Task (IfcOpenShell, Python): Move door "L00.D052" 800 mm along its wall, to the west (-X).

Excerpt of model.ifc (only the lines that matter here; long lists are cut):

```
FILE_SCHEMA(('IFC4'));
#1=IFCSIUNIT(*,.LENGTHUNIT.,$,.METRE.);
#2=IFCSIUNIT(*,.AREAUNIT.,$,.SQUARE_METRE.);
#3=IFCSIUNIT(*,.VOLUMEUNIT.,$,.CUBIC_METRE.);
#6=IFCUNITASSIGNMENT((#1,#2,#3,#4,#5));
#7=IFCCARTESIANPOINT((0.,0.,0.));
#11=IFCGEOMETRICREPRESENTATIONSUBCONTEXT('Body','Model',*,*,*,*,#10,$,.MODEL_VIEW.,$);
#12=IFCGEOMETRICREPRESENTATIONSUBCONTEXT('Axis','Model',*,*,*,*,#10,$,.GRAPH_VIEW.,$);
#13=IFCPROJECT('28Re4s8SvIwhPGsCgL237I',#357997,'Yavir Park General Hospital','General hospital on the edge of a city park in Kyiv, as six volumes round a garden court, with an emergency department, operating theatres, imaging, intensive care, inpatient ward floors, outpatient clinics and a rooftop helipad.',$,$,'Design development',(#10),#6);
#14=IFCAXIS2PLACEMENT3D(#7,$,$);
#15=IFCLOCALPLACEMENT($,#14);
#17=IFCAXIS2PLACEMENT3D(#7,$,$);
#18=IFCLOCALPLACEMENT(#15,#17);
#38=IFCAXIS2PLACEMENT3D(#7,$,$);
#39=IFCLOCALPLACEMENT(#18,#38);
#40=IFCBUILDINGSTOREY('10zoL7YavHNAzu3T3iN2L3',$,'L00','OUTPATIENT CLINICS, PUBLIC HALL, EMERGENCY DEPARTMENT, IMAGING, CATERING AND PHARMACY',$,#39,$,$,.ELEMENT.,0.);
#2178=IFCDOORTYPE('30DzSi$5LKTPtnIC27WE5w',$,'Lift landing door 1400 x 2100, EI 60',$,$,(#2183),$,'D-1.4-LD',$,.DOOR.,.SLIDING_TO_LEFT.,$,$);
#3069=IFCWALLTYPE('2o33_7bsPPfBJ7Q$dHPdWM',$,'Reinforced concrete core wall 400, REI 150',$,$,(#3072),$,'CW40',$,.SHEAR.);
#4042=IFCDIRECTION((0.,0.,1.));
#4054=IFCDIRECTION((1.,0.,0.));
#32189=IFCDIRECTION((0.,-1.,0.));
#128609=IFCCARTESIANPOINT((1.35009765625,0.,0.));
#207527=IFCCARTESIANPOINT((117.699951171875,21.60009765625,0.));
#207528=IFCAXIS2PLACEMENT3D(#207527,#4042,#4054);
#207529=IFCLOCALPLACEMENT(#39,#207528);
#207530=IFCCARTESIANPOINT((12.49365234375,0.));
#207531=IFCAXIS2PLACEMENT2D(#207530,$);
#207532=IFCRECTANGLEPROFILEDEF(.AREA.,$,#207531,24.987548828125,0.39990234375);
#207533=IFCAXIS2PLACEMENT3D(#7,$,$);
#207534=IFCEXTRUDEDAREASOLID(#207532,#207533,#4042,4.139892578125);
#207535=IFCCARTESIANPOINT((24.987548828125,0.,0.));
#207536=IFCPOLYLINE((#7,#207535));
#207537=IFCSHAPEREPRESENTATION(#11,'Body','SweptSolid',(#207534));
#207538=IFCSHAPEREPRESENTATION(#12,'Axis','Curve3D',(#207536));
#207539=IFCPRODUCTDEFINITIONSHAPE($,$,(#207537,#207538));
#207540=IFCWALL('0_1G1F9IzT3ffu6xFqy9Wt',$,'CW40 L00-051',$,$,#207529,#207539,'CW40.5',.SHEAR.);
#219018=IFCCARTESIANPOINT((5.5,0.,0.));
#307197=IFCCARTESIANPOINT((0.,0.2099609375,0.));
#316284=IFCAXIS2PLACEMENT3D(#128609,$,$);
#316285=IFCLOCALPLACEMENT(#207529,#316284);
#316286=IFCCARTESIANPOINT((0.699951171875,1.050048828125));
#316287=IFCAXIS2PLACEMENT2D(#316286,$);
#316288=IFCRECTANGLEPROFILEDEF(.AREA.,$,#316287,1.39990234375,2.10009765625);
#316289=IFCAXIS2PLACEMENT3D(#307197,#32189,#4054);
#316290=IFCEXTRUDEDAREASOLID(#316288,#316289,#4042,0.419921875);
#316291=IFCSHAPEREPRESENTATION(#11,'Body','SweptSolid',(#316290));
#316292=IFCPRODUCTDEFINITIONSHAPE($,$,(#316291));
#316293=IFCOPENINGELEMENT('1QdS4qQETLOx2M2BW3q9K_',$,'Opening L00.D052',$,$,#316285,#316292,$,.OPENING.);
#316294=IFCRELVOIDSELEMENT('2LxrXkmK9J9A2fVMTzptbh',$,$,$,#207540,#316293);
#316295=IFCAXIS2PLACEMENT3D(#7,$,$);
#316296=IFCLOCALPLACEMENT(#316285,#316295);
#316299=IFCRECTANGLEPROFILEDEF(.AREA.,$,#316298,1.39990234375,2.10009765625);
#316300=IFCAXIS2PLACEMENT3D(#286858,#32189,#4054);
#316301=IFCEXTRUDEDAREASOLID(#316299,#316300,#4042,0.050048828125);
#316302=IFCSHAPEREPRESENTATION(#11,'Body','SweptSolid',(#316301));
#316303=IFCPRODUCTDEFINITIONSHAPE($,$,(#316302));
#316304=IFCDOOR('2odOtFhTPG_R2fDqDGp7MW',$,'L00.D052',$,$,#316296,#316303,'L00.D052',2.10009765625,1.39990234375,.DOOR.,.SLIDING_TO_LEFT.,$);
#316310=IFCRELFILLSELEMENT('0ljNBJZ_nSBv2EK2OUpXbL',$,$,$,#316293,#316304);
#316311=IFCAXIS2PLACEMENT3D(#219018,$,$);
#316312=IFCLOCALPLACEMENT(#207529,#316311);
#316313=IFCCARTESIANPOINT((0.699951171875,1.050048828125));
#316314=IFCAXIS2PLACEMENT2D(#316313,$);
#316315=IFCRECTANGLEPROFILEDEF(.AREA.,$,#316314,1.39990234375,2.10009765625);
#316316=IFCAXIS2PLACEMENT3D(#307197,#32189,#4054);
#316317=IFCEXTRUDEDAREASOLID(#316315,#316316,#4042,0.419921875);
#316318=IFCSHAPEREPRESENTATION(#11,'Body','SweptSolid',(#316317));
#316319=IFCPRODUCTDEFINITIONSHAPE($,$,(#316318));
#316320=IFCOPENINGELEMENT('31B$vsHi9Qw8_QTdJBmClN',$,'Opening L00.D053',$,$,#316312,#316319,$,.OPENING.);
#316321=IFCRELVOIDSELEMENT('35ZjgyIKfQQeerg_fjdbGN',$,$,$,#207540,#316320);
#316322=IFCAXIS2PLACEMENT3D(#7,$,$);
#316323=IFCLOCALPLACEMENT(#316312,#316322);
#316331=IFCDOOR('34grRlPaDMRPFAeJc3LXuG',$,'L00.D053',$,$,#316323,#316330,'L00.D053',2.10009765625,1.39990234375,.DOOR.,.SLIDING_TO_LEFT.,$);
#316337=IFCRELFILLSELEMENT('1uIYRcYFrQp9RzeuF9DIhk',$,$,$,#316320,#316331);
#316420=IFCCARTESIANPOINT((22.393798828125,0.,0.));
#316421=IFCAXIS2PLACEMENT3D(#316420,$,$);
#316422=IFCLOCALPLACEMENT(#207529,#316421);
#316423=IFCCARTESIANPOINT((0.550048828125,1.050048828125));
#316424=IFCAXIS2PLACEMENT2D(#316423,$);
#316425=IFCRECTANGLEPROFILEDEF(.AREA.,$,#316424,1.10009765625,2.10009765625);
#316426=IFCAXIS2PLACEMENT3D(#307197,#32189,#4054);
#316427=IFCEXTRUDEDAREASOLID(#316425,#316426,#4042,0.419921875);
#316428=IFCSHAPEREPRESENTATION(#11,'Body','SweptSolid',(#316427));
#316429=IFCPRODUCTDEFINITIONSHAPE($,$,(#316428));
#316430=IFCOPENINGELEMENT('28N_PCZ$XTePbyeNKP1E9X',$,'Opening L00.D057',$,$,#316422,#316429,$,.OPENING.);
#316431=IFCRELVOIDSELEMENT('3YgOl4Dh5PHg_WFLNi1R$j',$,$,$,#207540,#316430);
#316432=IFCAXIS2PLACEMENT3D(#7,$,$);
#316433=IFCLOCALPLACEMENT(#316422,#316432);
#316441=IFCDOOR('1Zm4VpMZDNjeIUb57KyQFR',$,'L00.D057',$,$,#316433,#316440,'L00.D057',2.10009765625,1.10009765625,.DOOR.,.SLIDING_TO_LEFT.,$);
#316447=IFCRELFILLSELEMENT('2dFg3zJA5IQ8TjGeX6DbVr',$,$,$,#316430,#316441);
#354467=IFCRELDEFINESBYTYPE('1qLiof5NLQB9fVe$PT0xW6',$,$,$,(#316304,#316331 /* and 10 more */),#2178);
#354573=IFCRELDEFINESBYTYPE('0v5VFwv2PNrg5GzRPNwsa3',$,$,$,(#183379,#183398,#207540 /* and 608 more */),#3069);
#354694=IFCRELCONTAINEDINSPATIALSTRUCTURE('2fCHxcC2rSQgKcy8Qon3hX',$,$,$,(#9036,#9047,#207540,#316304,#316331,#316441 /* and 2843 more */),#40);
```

```python
import ifcopenshell
import ifcopenshell.api.geometry
import ifcopenshell.util.placement
import ifcopenshell.util.unit

model = ifcopenshell.open("model.ifc")
unit_scale = ifcopenshell.util.unit.calculate_unit_scale(model)

door = model.by_guid("2odOtFhTPG_R2fDqDGp7MW")
opening = door.FillsVoids[0].RelatingOpeningElement
wall = opening.VoidsElements[0].RelatingBuildingElement

wall_matrix = ifcopenshell.util.placement.get_local_placement(wall.ObjectPlacement)
shift = wall_matrix[:3, 0] * -0.8 / unit_scale
before = ifcopenshell.util.placement.get_local_placement(door.ObjectPlacement)[:3, 3].copy()

# The door is placed relative to its opening, so it follows when the opening moves.
matrix = ifcopenshell.util.placement.get_local_placement(opening.ObjectPlacement)
matrix[:3, 3] += shift
ifcopenshell.api.geometry.edit_object_placement(
    model, product=opening, matrix=matrix, is_si=False, should_transform_children=True
)

after = ifcopenshell.util.placement.get_local_placement(door.ObjectPlacement)[:3, 3]
print("door moved by", (after - before).round(3) + 0.0)

model.write("model_v2.ifc")
```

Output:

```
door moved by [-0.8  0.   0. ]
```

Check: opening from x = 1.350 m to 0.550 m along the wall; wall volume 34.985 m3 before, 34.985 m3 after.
